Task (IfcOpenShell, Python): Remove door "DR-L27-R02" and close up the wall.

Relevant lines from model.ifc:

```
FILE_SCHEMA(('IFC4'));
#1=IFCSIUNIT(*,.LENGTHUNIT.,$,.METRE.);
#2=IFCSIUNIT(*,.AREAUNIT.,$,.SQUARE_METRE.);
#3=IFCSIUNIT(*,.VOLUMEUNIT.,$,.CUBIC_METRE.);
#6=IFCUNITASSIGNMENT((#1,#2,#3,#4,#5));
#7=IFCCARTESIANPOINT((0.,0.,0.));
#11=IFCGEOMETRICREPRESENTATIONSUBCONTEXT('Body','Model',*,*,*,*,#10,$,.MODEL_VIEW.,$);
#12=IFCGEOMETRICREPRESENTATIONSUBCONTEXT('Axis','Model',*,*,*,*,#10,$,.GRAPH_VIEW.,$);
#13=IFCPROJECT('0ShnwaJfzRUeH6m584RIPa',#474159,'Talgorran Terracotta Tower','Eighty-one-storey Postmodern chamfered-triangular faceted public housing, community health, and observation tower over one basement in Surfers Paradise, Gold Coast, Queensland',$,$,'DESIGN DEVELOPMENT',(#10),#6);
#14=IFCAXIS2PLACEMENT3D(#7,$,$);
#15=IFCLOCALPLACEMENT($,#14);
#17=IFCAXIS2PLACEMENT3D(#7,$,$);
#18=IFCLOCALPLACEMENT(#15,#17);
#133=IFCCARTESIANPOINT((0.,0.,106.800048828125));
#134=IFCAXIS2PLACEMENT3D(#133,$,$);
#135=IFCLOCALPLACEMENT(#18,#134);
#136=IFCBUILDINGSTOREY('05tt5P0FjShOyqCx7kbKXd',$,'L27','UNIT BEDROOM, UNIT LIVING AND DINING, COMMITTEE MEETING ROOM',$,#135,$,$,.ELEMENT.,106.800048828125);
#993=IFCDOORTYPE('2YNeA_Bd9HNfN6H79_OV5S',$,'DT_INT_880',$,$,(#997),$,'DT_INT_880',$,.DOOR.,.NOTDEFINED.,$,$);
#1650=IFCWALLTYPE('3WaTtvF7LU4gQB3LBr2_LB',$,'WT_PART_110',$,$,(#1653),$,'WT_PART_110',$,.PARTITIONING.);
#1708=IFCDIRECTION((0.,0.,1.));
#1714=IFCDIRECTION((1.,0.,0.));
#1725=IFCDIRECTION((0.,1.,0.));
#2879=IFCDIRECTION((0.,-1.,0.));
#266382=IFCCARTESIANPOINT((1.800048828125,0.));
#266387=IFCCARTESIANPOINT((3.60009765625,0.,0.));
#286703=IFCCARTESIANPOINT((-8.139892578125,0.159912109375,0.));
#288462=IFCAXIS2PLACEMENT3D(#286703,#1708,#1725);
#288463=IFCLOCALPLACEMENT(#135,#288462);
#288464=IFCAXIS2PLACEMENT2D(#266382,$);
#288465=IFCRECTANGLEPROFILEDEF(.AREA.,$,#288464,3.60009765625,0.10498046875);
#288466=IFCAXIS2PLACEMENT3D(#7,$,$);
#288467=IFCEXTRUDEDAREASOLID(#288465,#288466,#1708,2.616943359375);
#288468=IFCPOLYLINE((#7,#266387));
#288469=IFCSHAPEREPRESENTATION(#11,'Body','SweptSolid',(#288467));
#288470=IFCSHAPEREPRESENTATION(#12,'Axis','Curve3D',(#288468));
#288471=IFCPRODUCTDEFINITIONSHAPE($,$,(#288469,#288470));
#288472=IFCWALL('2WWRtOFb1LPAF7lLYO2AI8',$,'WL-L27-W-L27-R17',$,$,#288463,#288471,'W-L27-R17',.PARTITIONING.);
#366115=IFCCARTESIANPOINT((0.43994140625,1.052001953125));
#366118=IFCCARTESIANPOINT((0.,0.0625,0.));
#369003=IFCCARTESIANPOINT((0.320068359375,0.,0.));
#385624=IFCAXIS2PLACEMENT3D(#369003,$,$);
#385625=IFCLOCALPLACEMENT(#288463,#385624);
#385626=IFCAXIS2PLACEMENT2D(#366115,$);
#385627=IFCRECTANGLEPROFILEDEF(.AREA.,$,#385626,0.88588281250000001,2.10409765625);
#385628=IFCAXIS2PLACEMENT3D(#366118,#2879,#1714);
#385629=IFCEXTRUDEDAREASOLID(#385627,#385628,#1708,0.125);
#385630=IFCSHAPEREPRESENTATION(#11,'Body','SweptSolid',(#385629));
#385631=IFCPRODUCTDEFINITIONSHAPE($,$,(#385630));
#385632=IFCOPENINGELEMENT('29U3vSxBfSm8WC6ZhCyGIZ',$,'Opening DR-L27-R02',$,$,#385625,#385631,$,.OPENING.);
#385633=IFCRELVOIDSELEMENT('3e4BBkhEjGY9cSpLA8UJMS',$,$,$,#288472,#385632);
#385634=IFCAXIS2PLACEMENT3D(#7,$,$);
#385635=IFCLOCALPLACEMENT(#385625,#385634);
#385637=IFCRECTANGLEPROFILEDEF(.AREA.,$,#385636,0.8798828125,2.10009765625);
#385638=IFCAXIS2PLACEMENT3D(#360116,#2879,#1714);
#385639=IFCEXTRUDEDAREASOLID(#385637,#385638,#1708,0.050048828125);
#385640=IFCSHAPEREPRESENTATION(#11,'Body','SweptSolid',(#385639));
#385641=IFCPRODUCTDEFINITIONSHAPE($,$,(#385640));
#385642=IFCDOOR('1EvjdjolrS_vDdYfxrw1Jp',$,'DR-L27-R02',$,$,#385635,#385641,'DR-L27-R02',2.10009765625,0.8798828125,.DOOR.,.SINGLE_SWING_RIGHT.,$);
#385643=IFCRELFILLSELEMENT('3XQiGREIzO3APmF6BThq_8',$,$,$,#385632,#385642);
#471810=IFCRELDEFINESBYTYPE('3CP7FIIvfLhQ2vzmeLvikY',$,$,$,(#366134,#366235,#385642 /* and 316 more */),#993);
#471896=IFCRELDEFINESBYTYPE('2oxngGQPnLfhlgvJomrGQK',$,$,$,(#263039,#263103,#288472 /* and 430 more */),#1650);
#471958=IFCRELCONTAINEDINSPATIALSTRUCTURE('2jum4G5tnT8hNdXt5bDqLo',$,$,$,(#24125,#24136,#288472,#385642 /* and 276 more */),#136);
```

```python
import ifcopenshell
import ifcopenshell.api.feature
import ifcopenshell.api.root
import ifcopenshell.geom
import ifcopenshell.util.shape

model = ifcopenshell.open("model.ifc")
settings = ifcopenshell.geom.settings()


def volume(element):
    """Net volume in cubic metres, openings subtracted."""
    shape = ifcopenshell.geom.create_shape(settings, element)
    return ifcopenshell.util.shape.get_volume(shape.geometry)


door = model.by_guid("1EvjdjolrS_vDdYfxrw1Jp")
opening = door.FillsVoids[0].RelatingOpeningElement
wall = opening.VoidsElements[0].RelatingBuildingElement
before = volume(wall)

ifcopenshell.api.root.remove_product(model, product=door)
ifcopenshell.api.feature.remove_feature(model, feature=opening)

after = volume(wall)

print(f"wall volume {before:.3f} -> {after:.3f} m3")

model.write("model-out.ifc")
```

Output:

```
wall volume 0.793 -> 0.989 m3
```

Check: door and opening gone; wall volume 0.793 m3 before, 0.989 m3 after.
